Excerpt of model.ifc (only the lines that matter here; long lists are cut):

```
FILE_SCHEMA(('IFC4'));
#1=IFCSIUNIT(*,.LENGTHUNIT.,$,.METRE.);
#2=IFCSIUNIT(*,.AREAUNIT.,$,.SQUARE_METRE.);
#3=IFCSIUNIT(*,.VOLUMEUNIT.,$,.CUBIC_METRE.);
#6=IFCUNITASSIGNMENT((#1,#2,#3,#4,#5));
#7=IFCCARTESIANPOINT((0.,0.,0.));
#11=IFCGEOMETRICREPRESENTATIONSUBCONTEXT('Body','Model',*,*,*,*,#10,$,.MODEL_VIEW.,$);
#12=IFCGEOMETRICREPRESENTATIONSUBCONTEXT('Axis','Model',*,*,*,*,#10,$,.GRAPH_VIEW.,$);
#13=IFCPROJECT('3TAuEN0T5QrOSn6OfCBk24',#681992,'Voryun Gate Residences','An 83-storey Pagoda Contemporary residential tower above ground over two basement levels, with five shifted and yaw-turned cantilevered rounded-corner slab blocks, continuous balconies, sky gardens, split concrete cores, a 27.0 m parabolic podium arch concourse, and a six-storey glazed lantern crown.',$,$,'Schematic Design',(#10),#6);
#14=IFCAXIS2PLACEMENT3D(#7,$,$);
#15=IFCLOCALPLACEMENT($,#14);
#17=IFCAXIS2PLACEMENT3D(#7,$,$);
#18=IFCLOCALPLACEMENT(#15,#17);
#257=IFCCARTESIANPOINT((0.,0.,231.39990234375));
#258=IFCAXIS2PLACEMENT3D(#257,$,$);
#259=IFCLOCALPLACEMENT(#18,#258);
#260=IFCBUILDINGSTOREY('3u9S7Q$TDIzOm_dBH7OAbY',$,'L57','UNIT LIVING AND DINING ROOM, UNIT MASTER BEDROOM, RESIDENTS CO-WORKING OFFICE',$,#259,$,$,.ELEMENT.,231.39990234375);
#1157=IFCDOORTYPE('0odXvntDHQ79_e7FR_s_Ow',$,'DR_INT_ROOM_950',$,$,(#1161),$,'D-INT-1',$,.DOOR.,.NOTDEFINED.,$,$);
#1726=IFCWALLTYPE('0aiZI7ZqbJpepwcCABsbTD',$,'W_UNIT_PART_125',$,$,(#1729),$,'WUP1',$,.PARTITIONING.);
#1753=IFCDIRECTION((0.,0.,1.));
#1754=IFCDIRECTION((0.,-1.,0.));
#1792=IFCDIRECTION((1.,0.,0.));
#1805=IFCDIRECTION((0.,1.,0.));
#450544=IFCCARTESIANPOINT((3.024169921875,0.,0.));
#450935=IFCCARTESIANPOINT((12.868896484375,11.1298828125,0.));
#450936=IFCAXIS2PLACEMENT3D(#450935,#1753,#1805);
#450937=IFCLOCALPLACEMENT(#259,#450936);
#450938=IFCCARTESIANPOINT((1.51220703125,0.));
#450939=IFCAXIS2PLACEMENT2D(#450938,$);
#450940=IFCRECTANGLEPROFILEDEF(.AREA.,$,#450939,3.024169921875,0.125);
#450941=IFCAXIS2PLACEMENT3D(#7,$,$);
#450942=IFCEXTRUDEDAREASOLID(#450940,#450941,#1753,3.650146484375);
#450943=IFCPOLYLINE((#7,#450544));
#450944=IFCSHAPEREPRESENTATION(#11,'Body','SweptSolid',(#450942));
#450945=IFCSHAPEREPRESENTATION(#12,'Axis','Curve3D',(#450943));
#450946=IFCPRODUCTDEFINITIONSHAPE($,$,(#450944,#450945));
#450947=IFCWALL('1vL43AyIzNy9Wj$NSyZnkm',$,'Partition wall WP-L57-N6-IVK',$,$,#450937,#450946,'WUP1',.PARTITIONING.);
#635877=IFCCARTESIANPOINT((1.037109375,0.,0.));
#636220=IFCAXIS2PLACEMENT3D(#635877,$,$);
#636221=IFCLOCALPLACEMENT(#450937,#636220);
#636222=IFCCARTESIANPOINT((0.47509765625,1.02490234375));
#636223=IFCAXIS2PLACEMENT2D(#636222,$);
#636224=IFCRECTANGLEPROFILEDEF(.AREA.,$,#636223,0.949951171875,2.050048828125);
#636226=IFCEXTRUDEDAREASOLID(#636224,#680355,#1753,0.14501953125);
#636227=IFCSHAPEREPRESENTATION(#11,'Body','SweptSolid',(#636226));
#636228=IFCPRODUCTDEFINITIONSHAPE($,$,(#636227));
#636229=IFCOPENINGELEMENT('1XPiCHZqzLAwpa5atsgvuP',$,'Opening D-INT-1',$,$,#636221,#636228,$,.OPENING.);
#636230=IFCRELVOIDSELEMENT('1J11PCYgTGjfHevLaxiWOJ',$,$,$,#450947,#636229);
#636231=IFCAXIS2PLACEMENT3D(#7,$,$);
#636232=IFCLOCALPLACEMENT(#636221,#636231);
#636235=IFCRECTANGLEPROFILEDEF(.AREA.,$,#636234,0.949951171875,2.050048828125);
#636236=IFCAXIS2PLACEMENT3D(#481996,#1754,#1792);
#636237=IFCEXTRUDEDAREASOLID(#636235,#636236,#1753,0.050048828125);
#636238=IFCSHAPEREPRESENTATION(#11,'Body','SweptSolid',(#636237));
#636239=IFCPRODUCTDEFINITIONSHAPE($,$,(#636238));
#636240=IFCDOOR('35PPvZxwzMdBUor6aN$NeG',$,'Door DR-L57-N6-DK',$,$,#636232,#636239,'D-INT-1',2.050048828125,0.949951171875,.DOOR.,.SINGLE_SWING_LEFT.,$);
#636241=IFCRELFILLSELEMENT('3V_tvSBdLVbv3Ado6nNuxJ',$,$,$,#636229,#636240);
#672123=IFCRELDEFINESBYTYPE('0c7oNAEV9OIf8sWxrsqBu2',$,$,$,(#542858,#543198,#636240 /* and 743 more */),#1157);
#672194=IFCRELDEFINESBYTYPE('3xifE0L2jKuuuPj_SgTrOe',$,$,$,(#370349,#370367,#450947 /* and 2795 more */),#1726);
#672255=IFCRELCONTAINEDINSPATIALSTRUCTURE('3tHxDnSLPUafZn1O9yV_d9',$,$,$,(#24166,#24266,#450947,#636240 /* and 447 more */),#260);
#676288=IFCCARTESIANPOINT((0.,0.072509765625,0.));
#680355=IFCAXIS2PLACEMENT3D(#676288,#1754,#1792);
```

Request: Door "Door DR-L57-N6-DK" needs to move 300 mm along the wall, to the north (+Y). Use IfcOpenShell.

```python
import ifcopenshell
import ifcopenshell.api.geometry
import ifcopenshell.util.placement
import ifcopenshell.util.unit

model = ifcopenshell.open("model.ifc")
unit_scale = ifcopenshell.util.unit.calculate_unit_scale(model)

door = model.by_guid("35PPvZxwzMdBUor6aN$NeG")
opening = door.FillsVoids[0].RelatingOpeningElement
wall = opening.VoidsElements[0].RelatingBuildingElement

wall_matrix = ifcopenshell.util.placement.get_local_placement(wall.ObjectPlacement)
shift = wall_matrix[:3, 0] * 0.3 / unit_scale
before = ifcopenshell.util.placement.get_local_placement(door.ObjectPlacement)[:3, 3].copy()

# The door is placed relative to its opening, so it follows when the opening moves.
matrix = ifcopenshell.util.placement.get_local_placement(opening.ObjectPlacement)
matrix[:3, 3] += shift
ifcopenshell.api.geometry.edit_object_placement(
    model, product=opening, matrix=matrix, is_si=False, should_transform_children=True
)

after = ifcopenshell.util.placement.get_local_placement(door.ObjectPlacement)[:3, 3]
print("door moved by", (after - before).round(3) + 0.0)

model.write("model_v2.ifc")
```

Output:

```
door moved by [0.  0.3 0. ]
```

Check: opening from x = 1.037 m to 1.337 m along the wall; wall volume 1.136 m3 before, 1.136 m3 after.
